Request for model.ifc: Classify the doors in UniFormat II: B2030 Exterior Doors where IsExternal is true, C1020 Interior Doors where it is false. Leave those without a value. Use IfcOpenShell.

First a look at what the model holds.

```python
import ifcopenshell
import ifcopenshell.util.element

model = ifcopenshell.open("model.ifc")
print(model.schema)
print("classifications:", [c.Name for c in model.by_type("IfcClassification")])
values = [ifcopenshell.util.element.get_pset(e, "Pset_DoorCommon", "IsExternal") for e in model.by_type("IfcDoor")]
for value in (True, False, None):
    print("IsExternal", value, values.count(value))
```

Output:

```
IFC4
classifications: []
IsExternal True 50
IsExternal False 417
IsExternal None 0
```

```python
import ifcopenshell
import ifcopenshell.api.classification
import ifcopenshell.util.element

model = ifcopenshell.open("model.ifc")

system = ifcopenshell.api.classification.add_classification(model, classification="UniFormat II")

doors = model.by_type("IfcDoor")
external = {e: ifcopenshell.util.element.get_pset(e, "Pset_DoorCommon", "IsExternal") for e in doors}
for flag, code, name in ((True, "B2030", "Exterior Doors"), (False, "C1020", "Interior Doors")):
    products = [e for e in doors if external[e] is flag]
    ifcopenshell.api.classification.add_reference(
        model, products=products, classification=system, identification=code, name=name
    )
    print(code, len(products))

model.write("model_edited.ifc")
```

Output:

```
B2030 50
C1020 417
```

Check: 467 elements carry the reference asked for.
